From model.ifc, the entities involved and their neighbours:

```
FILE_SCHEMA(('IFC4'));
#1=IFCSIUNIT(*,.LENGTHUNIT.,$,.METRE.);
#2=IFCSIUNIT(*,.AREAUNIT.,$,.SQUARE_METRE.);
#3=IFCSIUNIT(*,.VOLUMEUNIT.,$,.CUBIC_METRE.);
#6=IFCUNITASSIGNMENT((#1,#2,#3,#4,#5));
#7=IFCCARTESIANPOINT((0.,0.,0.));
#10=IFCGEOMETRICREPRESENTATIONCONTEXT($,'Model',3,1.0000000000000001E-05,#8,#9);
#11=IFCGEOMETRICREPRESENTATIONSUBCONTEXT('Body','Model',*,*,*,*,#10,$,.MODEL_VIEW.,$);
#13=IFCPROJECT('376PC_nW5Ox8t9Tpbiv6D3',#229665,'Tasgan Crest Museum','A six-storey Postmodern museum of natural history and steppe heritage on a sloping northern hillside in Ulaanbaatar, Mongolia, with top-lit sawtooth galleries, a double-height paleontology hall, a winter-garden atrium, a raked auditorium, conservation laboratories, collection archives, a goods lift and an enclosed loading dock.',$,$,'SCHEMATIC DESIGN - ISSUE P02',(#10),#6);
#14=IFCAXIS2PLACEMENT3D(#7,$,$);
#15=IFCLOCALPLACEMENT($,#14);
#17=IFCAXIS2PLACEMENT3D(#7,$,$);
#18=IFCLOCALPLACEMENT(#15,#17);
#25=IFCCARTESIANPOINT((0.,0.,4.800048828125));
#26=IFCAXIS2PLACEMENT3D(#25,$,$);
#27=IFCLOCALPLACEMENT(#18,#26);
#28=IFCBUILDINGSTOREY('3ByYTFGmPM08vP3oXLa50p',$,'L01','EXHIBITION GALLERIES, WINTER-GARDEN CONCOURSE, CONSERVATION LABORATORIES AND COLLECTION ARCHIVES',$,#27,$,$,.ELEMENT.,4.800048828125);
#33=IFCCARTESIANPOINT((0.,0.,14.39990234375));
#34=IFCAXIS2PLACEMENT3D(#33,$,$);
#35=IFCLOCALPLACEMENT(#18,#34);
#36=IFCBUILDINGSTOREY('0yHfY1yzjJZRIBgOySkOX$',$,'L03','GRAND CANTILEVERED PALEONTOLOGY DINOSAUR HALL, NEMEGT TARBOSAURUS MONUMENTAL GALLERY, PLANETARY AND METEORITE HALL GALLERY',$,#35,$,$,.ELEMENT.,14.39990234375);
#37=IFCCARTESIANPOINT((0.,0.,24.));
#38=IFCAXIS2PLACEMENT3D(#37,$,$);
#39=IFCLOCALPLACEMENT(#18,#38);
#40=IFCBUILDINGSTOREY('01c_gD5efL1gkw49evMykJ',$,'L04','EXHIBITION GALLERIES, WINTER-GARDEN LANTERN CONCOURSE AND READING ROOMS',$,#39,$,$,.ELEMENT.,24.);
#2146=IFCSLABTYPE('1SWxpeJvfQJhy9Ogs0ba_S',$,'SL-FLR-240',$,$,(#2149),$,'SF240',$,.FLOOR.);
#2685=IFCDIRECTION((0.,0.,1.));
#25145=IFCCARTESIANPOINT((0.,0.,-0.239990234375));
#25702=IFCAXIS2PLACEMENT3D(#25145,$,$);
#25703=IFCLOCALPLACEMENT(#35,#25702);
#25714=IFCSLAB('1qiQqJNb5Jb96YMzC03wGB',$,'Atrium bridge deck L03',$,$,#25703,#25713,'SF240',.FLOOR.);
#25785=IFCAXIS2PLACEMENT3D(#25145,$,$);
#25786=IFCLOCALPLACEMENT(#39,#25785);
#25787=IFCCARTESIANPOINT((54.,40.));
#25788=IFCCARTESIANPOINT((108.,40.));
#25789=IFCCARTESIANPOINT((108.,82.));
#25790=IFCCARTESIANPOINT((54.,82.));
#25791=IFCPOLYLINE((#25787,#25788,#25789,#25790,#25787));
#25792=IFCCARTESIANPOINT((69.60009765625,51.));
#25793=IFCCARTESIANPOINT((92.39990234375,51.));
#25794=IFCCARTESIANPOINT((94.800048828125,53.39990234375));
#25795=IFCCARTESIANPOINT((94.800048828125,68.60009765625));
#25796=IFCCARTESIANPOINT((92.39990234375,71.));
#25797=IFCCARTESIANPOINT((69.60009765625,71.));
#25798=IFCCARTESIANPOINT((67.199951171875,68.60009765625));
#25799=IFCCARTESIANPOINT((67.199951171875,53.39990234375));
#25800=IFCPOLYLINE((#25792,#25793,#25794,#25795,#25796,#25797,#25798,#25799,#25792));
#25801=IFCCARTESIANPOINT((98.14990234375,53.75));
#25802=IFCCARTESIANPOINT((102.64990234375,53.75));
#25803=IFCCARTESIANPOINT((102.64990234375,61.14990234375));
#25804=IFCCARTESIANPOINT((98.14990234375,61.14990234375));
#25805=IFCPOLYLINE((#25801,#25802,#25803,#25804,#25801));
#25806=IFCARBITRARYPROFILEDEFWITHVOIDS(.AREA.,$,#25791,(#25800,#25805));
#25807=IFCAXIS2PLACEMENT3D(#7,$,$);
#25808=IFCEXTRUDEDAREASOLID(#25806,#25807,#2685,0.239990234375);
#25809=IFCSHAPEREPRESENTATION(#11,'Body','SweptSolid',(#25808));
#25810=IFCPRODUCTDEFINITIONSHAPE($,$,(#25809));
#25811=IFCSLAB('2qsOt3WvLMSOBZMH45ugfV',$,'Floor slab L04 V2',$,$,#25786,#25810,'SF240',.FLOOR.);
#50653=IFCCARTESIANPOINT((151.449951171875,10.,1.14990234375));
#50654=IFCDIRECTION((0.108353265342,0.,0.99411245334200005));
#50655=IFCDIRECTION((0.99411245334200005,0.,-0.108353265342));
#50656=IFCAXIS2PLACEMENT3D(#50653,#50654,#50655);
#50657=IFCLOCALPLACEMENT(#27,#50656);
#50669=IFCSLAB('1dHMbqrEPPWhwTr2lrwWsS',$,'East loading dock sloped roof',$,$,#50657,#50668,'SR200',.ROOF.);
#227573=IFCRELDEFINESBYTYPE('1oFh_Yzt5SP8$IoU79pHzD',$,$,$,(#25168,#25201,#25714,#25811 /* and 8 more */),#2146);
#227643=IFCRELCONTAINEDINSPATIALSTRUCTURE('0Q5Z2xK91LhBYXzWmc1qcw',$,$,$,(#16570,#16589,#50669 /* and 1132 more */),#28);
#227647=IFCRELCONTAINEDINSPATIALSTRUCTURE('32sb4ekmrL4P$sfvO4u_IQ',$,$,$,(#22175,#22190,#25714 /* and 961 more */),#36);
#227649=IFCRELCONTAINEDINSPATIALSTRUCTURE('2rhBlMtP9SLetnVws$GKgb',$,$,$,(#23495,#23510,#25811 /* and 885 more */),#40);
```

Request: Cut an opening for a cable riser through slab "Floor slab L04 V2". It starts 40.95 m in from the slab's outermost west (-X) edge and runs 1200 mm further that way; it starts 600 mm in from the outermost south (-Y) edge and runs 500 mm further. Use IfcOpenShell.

```python
import numpy as np
import ifcopenshell
import ifcopenshell.api.feature
import ifcopenshell.api.geometry
import ifcopenshell.api.root
import ifcopenshell.geom
import ifcopenshell.util.placement
import ifcopenshell.util.representation
import ifcopenshell.util.shape
import ifcopenshell.util.unit

model = ifcopenshell.open("model.ifc")
unit_scale = ifcopenshell.util.unit.calculate_unit_scale(model)
settings = ifcopenshell.geom.settings()


def volume(element):
    """Net volume in cubic metres, openings subtracted."""
    shape = ifcopenshell.geom.create_shape(settings, element)
    return ifcopenshell.util.shape.get_volume(shape.geometry)


slab = model.by_id(25811)
before = volume(slab)

# Extent in the slab's own axes, in metres. The edges named are its -X and -Y sides.
slab_shape = ifcopenshell.geom.create_shape(settings, slab)
vertices = ifcopenshell.util.shape.get_vertices(slab_shape.geometry)
x_min, y_min, bottom = vertices.min(axis=0)
top = vertices[:, 2].max()

opening = ifcopenshell.api.root.create_entity(model, ifc_class="IfcOpeningElement", name="Cable riser opening", predefined_type="OPENING")
context = ifcopenshell.util.representation.get_context(model, "Model", "Body", "MODEL_VIEW")
width, depth = 1.2, 0.5
outline = [(0.0, 0.0), (width, 0.0), (width, depth), (0.0, depth), (0.0, 0.0)]
# Overshoot both faces by 50 mm so the cut is clean.
shape = ifcopenshell.api.geometry.add_slab_representation(
    model, context=context, depth=top - bottom + 0.1, polyline=outline
)
ifcopenshell.api.geometry.assign_representation(model, product=opening, representation=shape)

matrix = ifcopenshell.util.placement.get_local_placement(slab.ObjectPlacement)
matrix[:, 3] = matrix @ np.append(np.array([x_min + 40.95, y_min + 0.6, bottom - 0.05]) / unit_scale, 1.0)
ifcopenshell.api.geometry.edit_object_placement(model, product=opening, matrix=matrix, is_si=False)
ifcopenshell.api.feature.add_feature(model, feature=opening, element=slab)

after = volume(slab)

print(f"slab volume {before:.3f} -> {after:.3f} m3")

model.write("model_edited.ifc")
```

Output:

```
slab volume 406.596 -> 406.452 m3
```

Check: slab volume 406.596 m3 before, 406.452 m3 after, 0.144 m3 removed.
